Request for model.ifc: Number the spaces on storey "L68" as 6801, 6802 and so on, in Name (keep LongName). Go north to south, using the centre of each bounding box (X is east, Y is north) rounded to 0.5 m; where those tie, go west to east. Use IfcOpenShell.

First a look at what the model holds.

```python
import ifcopenshell
import ifcopenshell.util.element
import ifcopenshell.util.placement

model = ifcopenshell.open("model.ifc")
print(model.schema)
storey = next(s for s in model.by_type("IfcBuildingStorey") if s.Name == "L68")
spaces = [e for e in ifcopenshell.util.element.get_decomposition(storey) if e.is_a("IfcSpace")]
for e in sorted(spaces, key=lambda e: e.id()):
    origin = ifcopenshell.util.placement.get_local_placement(e.ObjectPlacement)[:3, 3]
    print(e.id(), e.Name, e.LongName, origin.round(2) + 0.0, sep=" | ")
```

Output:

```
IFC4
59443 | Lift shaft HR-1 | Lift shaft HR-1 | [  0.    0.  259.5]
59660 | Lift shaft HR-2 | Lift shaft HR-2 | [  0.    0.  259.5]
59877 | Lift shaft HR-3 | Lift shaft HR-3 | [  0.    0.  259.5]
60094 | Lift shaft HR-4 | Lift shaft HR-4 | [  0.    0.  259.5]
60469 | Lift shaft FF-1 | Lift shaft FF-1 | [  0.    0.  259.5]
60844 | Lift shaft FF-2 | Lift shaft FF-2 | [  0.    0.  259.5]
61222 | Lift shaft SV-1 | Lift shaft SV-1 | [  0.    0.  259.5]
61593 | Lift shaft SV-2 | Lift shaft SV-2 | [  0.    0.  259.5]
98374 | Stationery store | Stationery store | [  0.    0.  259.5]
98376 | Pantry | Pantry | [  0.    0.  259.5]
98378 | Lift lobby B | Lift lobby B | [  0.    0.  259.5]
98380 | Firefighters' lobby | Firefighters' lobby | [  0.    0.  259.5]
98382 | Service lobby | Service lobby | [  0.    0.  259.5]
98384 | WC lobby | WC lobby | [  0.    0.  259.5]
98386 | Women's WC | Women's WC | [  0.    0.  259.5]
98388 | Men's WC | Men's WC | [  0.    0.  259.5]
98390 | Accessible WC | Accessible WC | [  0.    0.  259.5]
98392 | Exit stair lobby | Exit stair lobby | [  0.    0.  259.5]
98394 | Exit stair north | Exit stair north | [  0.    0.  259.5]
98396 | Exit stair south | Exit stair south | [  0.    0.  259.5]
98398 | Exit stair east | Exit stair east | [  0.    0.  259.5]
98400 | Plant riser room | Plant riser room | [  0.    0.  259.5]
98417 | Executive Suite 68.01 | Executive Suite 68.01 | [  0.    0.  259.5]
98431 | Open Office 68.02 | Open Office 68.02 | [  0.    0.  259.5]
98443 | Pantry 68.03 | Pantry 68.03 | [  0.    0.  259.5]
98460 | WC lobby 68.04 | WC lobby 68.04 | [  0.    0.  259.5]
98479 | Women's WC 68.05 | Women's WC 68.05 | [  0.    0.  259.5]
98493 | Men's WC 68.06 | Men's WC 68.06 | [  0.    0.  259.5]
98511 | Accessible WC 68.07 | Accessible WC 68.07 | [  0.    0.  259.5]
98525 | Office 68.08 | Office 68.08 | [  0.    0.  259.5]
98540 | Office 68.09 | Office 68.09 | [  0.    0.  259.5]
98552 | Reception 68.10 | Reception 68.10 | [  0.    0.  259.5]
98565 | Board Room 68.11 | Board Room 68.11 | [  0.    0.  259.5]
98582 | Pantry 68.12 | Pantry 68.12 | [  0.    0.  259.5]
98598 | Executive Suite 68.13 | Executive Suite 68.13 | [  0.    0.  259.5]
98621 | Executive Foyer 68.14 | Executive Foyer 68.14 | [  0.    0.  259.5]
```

```python
import ifcopenshell
import ifcopenshell.geom
import ifcopenshell.util.element
import ifcopenshell.util.shape

model = ifcopenshell.open("model.ifc")
settings = ifcopenshell.geom.settings()
settings.set("use-world-coords", True)


def centre(element):
    shape = ifcopenshell.geom.create_shape(settings, element)
    return ifcopenshell.util.shape.get_bbox_centroid(shape.geometry)


storey = next(s for s in model.by_type("IfcBuildingStorey") if s.Name == "L68")
spaces = [e for e in ifcopenshell.util.element.get_decomposition(storey) if e.is_a("IfcSpace")]

# Insertion points can sit at a corner or the storey origin, so sort by the geometry (in metres).
centres = {e: centre(e) for e in spaces}
spaces.sort(key=lambda e: (-round(centres[e][1] / 0.5), centres[e][0]))

for i, e in enumerate(spaces, start=1):
    number = f"68{i:02d}"
    e.Name = number
    print(e.id(), number)

model.write("model_v2.ifc")
```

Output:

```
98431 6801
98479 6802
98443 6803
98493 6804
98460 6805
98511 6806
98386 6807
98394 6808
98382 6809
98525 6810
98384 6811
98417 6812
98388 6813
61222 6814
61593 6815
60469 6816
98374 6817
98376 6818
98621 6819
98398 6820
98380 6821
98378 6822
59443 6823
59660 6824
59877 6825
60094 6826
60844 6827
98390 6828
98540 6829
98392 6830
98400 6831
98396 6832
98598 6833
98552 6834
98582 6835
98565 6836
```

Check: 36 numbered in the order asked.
